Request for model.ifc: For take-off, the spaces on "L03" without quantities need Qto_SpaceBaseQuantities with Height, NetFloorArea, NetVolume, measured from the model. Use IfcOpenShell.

First a look at what the model holds.

```python
import ifcopenshell
import ifcopenshell.util.element
import ifcopenshell.util.unit

model = ifcopenshell.open("model.ifc")
print(model.schema)
for unit_type in ("LENGTHUNIT", "AREAUNIT", "VOLUMEUNIT"):
    print(unit_type, ifcopenshell.util.unit.calculate_unit_scale(model, unit_type))
storey = next(s for s in model.by_type("IfcBuildingStorey") if s.Name == "L03")
spaces = [e for e in ifcopenshell.util.element.get_decomposition(storey) if e.is_a("IfcSpace")]
for e in sorted(spaces, key=lambda e: e.id()):
    print(e.id(), e.is_a(), e.Name, list(ifcopenshell.util.element.get_psets(e, qtos_only=True)), sep=" | ")
```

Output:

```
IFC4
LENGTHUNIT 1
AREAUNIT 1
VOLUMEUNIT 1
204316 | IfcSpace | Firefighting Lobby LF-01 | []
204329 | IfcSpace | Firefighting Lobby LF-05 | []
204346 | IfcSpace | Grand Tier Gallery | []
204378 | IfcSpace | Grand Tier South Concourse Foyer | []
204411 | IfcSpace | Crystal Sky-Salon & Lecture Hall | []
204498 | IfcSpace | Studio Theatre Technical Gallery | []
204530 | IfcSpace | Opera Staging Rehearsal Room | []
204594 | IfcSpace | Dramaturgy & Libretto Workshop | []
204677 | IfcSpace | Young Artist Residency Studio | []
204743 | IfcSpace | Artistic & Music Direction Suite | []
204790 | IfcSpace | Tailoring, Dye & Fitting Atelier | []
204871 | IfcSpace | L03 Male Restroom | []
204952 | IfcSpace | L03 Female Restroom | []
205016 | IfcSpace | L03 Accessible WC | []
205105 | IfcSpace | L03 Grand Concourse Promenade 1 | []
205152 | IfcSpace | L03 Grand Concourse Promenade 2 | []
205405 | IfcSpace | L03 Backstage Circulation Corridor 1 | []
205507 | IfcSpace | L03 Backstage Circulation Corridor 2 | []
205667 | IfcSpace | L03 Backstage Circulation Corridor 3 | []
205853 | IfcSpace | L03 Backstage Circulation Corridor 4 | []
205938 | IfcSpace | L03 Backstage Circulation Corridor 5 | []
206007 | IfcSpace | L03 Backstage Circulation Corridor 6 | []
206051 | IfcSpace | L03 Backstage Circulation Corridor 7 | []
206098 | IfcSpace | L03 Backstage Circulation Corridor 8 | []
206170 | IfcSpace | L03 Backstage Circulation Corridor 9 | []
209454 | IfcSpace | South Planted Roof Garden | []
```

```python
import ifcopenshell
import ifcopenshell.api.pset
import ifcopenshell.geom
import ifcopenshell.util.element
import ifcopenshell.util.shape
import ifcopenshell.util.unit

model = ifcopenshell.open("model.ifc")
unit_scale = ifcopenshell.util.unit.calculate_unit_scale(model)
area_scale = ifcopenshell.util.unit.calculate_unit_scale(model, "AREAUNIT")
volume_scale = ifcopenshell.util.unit.calculate_unit_scale(model, "VOLUMEUNIT")
settings = ifcopenshell.geom.settings()

storey = next(s for s in model.by_type("IfcBuildingStorey") if s.Name == "L03")
spaces = [e for e in ifcopenshell.util.element.get_decomposition(storey) if e.is_a("IfcSpace")]

for e in sorted(spaces, key=lambda e: e.id()):
    if ifcopenshell.util.element.get_psets(e, qtos_only=True, should_inherit=False):
        continue
    # Geometry comes back in metres, in the element's own axes.
    shape = ifcopenshell.geom.create_shape(settings, e)
    values = {
        "Height": ifcopenshell.util.shape.get_z(shape.geometry) / unit_scale,
        "NetFloorArea": ifcopenshell.util.shape.get_footprint_area(shape.geometry) / area_scale,
        "NetVolume": ifcopenshell.util.shape.get_volume(shape.geometry) / volume_scale,
    }
    qto = ifcopenshell.api.pset.add_qto(model, product=e, name="Qto_SpaceBaseQuantities")
    ifcopenshell.api.pset.edit_qto(model, qto=qto, properties=values)
    print(e.id(), {k: round(v, 3) for k, v in values.items()})

model.write("model_updated.ifc")
```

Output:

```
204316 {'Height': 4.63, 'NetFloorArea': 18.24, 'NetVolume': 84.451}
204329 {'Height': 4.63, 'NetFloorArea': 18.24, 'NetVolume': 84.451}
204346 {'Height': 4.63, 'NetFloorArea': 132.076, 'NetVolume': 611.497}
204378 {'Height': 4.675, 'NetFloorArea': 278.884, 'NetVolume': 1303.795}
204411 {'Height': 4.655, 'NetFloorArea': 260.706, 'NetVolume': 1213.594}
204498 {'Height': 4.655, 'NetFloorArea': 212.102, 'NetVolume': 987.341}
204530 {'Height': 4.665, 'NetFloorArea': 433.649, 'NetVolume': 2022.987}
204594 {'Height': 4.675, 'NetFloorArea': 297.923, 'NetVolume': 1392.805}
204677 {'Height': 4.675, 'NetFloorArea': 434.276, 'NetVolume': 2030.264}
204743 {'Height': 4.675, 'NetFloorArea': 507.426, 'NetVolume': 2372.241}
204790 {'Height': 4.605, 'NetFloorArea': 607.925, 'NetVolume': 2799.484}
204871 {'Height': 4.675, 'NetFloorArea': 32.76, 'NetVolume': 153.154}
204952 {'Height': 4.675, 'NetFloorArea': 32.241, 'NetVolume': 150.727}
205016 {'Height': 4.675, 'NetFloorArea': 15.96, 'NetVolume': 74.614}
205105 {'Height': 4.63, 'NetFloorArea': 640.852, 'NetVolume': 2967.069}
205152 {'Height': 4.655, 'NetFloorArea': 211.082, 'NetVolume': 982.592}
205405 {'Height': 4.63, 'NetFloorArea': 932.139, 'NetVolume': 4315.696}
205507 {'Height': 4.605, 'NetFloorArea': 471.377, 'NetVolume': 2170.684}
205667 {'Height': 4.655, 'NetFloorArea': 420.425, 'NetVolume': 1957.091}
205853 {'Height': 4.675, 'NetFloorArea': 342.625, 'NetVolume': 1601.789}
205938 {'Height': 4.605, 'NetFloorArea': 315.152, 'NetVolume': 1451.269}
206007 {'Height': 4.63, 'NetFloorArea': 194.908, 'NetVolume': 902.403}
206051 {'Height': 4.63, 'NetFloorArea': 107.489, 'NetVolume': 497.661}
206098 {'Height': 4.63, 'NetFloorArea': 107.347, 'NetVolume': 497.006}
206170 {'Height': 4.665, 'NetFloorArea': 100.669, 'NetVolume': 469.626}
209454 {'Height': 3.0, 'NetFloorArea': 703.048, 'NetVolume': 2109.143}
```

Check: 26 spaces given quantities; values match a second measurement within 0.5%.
